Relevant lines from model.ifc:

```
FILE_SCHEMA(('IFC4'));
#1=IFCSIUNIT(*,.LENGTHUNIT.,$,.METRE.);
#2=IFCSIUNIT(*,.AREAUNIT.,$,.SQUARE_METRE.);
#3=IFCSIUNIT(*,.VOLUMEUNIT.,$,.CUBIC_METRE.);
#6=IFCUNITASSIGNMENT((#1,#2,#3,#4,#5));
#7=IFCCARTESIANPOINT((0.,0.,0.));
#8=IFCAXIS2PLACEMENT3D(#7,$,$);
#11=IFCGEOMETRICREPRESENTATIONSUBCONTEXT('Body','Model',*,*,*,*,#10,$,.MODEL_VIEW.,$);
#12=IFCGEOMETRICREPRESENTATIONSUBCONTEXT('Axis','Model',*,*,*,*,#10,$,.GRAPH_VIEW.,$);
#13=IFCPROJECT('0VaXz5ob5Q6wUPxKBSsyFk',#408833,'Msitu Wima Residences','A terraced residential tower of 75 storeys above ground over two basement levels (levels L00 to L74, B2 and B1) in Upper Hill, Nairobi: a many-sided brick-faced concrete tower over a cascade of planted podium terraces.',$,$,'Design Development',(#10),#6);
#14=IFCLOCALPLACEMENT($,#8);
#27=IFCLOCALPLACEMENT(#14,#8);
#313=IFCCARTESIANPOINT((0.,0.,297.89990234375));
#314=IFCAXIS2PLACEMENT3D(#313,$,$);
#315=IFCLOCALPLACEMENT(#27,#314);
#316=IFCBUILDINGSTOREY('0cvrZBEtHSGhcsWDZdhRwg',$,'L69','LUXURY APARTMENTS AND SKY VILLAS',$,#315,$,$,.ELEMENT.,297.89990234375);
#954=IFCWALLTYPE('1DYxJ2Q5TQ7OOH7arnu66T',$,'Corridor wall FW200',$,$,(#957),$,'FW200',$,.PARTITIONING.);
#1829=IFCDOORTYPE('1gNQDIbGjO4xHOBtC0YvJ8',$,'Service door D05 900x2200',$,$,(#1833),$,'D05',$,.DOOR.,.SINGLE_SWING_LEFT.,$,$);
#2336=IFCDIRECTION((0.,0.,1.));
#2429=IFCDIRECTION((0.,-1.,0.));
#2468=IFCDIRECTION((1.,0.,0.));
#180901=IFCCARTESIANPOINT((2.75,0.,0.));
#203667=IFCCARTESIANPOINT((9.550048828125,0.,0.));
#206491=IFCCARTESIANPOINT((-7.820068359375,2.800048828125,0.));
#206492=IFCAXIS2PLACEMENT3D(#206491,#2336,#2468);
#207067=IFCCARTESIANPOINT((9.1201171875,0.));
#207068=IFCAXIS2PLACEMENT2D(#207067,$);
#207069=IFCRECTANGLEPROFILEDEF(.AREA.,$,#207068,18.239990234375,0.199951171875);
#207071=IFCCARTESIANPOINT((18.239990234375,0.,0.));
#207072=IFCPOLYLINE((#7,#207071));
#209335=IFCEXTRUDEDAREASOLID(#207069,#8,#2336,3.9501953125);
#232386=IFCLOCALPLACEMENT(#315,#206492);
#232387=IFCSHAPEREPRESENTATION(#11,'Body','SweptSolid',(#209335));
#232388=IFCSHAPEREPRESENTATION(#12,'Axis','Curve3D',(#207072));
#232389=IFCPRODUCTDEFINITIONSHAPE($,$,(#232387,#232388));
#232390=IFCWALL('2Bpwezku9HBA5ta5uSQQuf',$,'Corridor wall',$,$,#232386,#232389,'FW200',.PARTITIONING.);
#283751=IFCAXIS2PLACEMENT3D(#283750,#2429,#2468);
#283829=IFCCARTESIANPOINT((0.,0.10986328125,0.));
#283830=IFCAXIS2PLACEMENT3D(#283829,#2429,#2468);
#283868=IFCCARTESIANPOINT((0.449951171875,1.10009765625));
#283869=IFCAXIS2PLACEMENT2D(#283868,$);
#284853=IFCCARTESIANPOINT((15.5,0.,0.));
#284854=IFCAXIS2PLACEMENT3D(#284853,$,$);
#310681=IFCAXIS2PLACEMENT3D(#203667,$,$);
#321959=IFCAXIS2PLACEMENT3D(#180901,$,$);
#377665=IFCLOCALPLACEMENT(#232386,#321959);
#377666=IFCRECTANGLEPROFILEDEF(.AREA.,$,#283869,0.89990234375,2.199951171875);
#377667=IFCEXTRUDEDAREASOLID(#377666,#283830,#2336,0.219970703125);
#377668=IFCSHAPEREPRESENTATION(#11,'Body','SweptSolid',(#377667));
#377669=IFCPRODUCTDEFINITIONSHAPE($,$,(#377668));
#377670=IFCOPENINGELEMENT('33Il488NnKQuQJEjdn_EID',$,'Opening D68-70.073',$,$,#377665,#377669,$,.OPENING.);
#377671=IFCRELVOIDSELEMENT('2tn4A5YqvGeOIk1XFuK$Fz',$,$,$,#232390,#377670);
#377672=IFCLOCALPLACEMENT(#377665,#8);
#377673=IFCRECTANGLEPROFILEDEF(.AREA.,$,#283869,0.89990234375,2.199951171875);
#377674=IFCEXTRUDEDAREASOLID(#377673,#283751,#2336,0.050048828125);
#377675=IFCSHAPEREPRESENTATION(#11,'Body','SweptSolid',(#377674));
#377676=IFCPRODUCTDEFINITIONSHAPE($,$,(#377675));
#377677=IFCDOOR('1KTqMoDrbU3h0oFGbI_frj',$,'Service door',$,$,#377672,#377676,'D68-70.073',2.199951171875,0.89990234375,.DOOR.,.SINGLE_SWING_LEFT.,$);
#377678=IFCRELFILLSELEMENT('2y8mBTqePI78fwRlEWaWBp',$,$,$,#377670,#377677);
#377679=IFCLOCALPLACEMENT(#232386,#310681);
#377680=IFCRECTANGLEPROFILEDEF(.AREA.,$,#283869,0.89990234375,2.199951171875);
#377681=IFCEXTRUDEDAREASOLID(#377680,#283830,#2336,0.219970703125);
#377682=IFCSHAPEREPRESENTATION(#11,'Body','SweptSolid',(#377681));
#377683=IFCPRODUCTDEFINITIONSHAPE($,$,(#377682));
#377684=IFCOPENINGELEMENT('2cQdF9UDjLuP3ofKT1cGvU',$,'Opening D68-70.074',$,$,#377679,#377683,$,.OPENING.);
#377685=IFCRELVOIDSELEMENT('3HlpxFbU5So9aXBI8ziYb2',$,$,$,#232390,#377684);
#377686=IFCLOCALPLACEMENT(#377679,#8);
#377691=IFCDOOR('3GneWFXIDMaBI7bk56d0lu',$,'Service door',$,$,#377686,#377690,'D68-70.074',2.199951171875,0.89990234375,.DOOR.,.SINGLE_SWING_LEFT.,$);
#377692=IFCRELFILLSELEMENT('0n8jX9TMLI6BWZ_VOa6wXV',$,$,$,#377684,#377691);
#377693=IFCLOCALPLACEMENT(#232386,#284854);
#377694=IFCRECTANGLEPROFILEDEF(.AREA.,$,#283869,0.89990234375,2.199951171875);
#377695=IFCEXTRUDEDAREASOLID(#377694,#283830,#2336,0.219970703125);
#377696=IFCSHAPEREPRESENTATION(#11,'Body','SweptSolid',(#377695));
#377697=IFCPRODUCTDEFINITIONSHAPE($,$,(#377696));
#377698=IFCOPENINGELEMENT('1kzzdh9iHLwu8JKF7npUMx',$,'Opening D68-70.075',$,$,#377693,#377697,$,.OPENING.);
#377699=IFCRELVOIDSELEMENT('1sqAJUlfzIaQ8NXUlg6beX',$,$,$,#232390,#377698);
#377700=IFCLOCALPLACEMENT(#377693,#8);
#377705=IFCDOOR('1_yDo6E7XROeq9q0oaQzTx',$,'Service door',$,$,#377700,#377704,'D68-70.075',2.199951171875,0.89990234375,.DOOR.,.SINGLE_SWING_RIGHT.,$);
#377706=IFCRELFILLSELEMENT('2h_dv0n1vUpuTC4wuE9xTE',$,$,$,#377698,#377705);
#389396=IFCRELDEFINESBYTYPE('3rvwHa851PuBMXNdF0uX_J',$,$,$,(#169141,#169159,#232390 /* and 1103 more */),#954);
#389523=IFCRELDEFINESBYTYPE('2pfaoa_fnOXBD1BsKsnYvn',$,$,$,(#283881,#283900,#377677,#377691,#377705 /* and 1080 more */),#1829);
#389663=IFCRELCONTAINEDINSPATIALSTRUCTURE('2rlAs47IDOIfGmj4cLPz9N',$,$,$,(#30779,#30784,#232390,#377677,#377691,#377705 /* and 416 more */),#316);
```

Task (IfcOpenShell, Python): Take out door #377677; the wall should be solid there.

```python
import ifcopenshell
import ifcopenshell.api.feature
import ifcopenshell.api.root
import ifcopenshell.geom
import ifcopenshell.util.shape

model = ifcopenshell.open("model.ifc")
settings = ifcopenshell.geom.settings()


def volume(element):
    """Net volume in cubic metres, openings subtracted."""
    shape = ifcopenshell.geom.create_shape(settings, element)
    return ifcopenshell.util.shape.get_volume(shape.geometry)


door = model.by_id(377677)
opening = door.FillsVoids[0].RelatingOpeningElement
wall = opening.VoidsElements[0].RelatingBuildingElement
before = volume(wall)

ifcopenshell.api.root.remove_product(model, product=door)
ifcopenshell.api.feature.remove_feature(model, feature=opening)

after = volume(wall)

print(f"wall volume {before:.3f} -> {after:.3f} m3")

model.write("model_rev.ifc")
```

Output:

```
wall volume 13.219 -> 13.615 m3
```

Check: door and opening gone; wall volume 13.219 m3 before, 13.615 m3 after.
